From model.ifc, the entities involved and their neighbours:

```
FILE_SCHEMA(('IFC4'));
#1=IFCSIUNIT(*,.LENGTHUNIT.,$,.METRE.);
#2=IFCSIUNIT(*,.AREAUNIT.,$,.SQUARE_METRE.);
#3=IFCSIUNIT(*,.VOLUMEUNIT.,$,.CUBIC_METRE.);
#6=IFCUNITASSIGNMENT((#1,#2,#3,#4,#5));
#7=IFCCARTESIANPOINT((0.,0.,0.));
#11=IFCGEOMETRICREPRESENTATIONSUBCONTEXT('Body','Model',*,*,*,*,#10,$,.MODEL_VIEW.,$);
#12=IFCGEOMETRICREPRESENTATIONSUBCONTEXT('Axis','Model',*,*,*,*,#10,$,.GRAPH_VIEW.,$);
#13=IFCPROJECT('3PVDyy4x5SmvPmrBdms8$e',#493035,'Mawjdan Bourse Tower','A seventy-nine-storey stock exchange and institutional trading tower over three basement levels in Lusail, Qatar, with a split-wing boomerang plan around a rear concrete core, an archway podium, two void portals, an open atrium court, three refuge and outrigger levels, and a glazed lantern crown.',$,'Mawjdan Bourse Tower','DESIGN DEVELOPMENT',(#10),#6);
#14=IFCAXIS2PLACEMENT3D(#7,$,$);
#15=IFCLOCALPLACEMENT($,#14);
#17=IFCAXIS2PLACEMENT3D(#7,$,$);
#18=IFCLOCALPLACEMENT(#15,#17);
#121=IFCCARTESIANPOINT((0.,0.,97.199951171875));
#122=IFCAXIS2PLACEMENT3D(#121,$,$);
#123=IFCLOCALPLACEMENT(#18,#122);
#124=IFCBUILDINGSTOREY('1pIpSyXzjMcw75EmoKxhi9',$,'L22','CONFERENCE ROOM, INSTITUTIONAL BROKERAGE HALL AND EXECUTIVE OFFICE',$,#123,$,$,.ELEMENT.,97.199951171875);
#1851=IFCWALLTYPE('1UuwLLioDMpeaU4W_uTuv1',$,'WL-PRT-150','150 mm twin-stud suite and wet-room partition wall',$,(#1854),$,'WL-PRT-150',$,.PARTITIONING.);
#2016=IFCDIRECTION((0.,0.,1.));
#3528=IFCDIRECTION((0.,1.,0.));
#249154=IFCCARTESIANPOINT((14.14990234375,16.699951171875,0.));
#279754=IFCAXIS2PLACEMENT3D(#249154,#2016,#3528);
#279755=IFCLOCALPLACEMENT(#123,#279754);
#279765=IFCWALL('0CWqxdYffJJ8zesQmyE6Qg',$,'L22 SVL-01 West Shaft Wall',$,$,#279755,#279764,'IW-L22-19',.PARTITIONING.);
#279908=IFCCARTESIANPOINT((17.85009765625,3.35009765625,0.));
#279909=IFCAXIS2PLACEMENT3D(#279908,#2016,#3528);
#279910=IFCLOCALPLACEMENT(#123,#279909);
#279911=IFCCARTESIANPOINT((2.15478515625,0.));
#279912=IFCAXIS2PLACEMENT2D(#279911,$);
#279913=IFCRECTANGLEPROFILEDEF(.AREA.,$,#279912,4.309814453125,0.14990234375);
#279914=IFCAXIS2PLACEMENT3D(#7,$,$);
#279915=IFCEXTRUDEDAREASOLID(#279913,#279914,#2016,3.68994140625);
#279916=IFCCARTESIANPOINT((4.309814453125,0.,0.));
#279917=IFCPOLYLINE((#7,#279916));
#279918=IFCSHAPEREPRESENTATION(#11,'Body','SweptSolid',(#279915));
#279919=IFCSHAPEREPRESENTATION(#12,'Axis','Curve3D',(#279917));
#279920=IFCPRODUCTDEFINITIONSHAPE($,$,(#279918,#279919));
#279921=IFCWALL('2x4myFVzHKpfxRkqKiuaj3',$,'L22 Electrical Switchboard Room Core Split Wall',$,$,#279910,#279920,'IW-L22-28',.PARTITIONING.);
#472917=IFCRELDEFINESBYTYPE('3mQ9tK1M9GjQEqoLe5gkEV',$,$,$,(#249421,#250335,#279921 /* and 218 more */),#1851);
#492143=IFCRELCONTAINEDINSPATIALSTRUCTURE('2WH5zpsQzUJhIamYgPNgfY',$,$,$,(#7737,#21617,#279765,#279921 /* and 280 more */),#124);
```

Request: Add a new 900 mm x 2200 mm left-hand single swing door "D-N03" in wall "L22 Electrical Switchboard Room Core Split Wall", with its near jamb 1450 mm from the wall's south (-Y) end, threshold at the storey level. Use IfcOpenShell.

```python
import numpy as np
import ifcopenshell
import ifcopenshell.api.feature
import ifcopenshell.api.geometry
import ifcopenshell.api.root
import ifcopenshell.api.spatial
import ifcopenshell.geom
import ifcopenshell.util.element
import ifcopenshell.util.placement
import ifcopenshell.util.representation
import ifcopenshell.util.shape
import ifcopenshell.util.unit

model = ifcopenshell.open("model.ifc")
unit_scale = ifcopenshell.util.unit.calculate_unit_scale(model)
settings = ifcopenshell.geom.settings()


def volume(element):
    """Net volume in cubic metres, openings subtracted."""
    shape = ifcopenshell.geom.create_shape(settings, element)
    return ifcopenshell.util.shape.get_volume(shape.geometry)


wall = model.by_guid("2x4myFVzHKpfxRkqKiuaj3")
storey = ifcopenshell.util.element.get_container(wall, ifc_class="IfcBuildingStorey")
context = ifcopenshell.util.representation.get_context(model, "Model", "Body", "MODEL_VIEW")
before = volume(wall)

width, height, from_end, sill = 0.9, 2.2, 1.45, 0.0  # metres

# The wall runs along its own X axis, and the end named is its -X end.
wall_shape = ifcopenshell.geom.create_shape(settings, wall)
x, y, z = ifcopenshell.util.shape.get_vertices(wall_shape.geometry).T
start = x.min() + from_end
face, thickness = float(y.min()), float(y.max() - y.min())
wall_matrix = ifcopenshell.util.placement.get_local_placement(wall.ObjectPlacement)
level = ifcopenshell.util.placement.get_local_placement(storey.ObjectPlacement)[2, 3]


def in_wall(x, y):
    """Placement at x, y metres in the wall's axes, at sill height."""
    matrix = wall_matrix.copy()
    matrix[:, 3] = wall_matrix @ np.array([x / unit_scale, y / unit_scale, 0.0, 1.0])
    matrix[2, 3] = level + sill / unit_scale
    return matrix


# Opening: a box that overshoots both wall faces by 50 mm.
opening = ifcopenshell.api.root.create_entity(model, ifc_class="IfcOpeningElement", predefined_type="OPENING")
box = ifcopenshell.api.geometry.add_wall_representation(
    model, context=context, length=width, height=height, thickness=thickness + 0.1
)
ifcopenshell.api.geometry.assign_representation(model, product=opening, representation=box)
ifcopenshell.api.geometry.edit_object_placement(model, product=opening, matrix=in_wall(start, face - 0.05), is_si=False)
ifcopenshell.api.feature.add_feature(model, feature=opening, element=wall)

door = ifcopenshell.api.root.create_entity(model, ifc_class="IfcDoor", name="D-N03", predefined_type="DOOR")
door.OverallWidth, door.OverallHeight = width / unit_scale, height / unit_scale
door.OperationType = "SINGLE_SWING_LEFT"
body = ifcopenshell.api.geometry.add_door_representation(
    model,
    context=context,
    overall_width=door.OverallWidth,
    overall_height=door.OverallHeight,
    operation_type="SINGLE_SWING_LEFT",
    lining_properties={"LiningDepth": thickness / unit_scale, "ThresholdDepth": thickness / unit_scale},
)
ifcopenshell.api.geometry.assign_representation(model, product=door, representation=body)
ifcopenshell.api.spatial.assign_container(model, products=[door], relating_structure=storey)
ifcopenshell.api.feature.add_filling(model, opening=opening, element=door)

# The lining spans the wall, so the door starts at the wall face.
ifcopenshell.api.geometry.edit_object_placement(model, product=door, matrix=in_wall(start, face), is_si=False)

after = volume(wall)

print(f"wall volume {before:.3f} -> {after:.3f} m3")

model.write("model_rev.ifc")
```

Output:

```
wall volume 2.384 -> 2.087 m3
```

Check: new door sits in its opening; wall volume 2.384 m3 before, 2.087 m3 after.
